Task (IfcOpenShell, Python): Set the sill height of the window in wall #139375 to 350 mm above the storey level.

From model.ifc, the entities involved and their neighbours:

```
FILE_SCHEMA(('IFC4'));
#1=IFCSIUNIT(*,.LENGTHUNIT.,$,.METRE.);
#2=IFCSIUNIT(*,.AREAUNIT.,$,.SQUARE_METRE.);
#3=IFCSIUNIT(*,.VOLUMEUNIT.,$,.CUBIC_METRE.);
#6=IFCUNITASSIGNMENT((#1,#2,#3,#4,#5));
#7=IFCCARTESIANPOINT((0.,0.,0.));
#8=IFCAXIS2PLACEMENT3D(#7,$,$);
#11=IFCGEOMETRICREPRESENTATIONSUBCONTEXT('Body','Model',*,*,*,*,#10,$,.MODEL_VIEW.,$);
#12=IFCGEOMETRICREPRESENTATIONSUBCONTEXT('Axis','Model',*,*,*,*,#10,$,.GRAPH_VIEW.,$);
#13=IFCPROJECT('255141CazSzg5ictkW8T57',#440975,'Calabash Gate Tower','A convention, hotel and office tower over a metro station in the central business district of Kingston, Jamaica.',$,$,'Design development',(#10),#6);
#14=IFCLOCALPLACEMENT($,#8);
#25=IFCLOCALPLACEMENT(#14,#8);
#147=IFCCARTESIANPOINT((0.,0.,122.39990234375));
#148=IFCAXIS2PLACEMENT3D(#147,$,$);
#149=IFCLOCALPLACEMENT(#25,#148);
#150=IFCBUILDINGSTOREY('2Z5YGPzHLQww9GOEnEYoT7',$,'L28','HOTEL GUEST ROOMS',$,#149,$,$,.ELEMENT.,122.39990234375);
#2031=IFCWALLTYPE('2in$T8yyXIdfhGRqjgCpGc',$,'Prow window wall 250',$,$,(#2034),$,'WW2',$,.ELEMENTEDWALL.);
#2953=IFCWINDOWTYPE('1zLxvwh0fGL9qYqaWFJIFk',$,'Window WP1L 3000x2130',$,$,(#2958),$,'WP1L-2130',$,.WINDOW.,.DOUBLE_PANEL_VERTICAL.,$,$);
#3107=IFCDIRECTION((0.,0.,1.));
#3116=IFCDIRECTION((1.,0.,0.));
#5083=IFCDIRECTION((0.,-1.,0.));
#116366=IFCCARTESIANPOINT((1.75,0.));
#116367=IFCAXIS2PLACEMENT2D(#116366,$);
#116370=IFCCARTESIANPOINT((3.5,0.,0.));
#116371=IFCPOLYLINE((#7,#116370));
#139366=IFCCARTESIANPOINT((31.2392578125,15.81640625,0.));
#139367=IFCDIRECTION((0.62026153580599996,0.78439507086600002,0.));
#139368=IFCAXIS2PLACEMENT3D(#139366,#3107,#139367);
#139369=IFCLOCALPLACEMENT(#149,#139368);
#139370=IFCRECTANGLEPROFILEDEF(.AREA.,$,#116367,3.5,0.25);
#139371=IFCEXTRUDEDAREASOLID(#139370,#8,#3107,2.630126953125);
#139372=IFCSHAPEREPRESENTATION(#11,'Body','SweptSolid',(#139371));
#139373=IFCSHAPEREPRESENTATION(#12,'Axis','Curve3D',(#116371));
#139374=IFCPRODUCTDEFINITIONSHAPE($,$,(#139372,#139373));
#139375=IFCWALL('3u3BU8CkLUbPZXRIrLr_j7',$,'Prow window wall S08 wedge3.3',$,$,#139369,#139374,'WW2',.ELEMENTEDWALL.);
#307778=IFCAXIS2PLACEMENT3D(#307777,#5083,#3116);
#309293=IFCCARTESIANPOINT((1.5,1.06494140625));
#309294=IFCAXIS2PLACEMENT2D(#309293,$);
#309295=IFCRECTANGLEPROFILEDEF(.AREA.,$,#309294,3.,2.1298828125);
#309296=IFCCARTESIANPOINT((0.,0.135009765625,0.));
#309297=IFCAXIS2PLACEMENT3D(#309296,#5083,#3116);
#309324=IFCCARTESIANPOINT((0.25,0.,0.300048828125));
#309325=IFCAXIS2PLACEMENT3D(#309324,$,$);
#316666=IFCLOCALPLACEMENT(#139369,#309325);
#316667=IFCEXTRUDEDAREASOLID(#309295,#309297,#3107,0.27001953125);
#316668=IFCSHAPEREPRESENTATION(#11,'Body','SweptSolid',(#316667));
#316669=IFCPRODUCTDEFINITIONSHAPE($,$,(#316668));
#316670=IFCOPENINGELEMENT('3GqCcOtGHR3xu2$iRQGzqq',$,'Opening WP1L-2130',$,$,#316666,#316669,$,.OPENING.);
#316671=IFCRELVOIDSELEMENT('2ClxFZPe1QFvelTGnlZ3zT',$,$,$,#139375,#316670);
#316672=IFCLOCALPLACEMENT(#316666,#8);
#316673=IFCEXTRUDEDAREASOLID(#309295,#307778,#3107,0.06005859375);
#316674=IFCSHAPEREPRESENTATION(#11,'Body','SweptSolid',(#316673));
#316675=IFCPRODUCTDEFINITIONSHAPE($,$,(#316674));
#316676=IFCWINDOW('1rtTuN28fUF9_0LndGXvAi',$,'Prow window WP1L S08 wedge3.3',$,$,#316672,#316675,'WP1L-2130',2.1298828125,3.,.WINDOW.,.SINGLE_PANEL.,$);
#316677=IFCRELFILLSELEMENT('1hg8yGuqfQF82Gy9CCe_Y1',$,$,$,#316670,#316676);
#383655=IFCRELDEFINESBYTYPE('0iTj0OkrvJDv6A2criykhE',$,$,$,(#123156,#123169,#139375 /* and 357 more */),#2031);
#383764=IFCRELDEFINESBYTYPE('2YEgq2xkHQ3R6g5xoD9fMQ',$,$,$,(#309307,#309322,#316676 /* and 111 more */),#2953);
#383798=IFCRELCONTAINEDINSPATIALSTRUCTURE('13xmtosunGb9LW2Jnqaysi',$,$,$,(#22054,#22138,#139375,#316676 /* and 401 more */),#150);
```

```python
import numpy as np
import ifcopenshell
import ifcopenshell.api.geometry
import ifcopenshell.geom
import ifcopenshell.util.element
import ifcopenshell.util.placement
import ifcopenshell.util.shape
import ifcopenshell.util.unit

model = ifcopenshell.open("model.ifc")
unit_scale = ifcopenshell.util.unit.calculate_unit_scale(model)

window = model.by_id(316676)
opening = window.FillsVoids[0].RelatingOpeningElement
storey = ifcopenshell.util.element.get_container(window, ifc_class="IfcBuildingStorey")
level = ifcopenshell.util.placement.get_local_placement(storey.ObjectPlacement)[2, 3]

# The opening's origin need not be at the sill, so measure its lowest point.
shape = ifcopenshell.geom.create_shape(ifcopenshell.geom.settings(), opening)
bottom = ifcopenshell.util.shape.get_shape_bottom_elevation(shape, shape.geometry) / unit_scale
dz = level + 0.35 / unit_scale - bottom

shift = np.array([0.0, 0.0, dz])
# The window is placed relative to its opening, so it follows when the opening moves.
matrix = ifcopenshell.util.placement.get_local_placement(opening.ObjectPlacement)
matrix[:3, 3] += shift
ifcopenshell.api.geometry.edit_object_placement(
    model, product=opening, matrix=matrix, is_si=False, should_transform_children=True
)

print(f"moved by {dz * unit_scale:+.3f} m")

model.write("model_rev.ifc")
```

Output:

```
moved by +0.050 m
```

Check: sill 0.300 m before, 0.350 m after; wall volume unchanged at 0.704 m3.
